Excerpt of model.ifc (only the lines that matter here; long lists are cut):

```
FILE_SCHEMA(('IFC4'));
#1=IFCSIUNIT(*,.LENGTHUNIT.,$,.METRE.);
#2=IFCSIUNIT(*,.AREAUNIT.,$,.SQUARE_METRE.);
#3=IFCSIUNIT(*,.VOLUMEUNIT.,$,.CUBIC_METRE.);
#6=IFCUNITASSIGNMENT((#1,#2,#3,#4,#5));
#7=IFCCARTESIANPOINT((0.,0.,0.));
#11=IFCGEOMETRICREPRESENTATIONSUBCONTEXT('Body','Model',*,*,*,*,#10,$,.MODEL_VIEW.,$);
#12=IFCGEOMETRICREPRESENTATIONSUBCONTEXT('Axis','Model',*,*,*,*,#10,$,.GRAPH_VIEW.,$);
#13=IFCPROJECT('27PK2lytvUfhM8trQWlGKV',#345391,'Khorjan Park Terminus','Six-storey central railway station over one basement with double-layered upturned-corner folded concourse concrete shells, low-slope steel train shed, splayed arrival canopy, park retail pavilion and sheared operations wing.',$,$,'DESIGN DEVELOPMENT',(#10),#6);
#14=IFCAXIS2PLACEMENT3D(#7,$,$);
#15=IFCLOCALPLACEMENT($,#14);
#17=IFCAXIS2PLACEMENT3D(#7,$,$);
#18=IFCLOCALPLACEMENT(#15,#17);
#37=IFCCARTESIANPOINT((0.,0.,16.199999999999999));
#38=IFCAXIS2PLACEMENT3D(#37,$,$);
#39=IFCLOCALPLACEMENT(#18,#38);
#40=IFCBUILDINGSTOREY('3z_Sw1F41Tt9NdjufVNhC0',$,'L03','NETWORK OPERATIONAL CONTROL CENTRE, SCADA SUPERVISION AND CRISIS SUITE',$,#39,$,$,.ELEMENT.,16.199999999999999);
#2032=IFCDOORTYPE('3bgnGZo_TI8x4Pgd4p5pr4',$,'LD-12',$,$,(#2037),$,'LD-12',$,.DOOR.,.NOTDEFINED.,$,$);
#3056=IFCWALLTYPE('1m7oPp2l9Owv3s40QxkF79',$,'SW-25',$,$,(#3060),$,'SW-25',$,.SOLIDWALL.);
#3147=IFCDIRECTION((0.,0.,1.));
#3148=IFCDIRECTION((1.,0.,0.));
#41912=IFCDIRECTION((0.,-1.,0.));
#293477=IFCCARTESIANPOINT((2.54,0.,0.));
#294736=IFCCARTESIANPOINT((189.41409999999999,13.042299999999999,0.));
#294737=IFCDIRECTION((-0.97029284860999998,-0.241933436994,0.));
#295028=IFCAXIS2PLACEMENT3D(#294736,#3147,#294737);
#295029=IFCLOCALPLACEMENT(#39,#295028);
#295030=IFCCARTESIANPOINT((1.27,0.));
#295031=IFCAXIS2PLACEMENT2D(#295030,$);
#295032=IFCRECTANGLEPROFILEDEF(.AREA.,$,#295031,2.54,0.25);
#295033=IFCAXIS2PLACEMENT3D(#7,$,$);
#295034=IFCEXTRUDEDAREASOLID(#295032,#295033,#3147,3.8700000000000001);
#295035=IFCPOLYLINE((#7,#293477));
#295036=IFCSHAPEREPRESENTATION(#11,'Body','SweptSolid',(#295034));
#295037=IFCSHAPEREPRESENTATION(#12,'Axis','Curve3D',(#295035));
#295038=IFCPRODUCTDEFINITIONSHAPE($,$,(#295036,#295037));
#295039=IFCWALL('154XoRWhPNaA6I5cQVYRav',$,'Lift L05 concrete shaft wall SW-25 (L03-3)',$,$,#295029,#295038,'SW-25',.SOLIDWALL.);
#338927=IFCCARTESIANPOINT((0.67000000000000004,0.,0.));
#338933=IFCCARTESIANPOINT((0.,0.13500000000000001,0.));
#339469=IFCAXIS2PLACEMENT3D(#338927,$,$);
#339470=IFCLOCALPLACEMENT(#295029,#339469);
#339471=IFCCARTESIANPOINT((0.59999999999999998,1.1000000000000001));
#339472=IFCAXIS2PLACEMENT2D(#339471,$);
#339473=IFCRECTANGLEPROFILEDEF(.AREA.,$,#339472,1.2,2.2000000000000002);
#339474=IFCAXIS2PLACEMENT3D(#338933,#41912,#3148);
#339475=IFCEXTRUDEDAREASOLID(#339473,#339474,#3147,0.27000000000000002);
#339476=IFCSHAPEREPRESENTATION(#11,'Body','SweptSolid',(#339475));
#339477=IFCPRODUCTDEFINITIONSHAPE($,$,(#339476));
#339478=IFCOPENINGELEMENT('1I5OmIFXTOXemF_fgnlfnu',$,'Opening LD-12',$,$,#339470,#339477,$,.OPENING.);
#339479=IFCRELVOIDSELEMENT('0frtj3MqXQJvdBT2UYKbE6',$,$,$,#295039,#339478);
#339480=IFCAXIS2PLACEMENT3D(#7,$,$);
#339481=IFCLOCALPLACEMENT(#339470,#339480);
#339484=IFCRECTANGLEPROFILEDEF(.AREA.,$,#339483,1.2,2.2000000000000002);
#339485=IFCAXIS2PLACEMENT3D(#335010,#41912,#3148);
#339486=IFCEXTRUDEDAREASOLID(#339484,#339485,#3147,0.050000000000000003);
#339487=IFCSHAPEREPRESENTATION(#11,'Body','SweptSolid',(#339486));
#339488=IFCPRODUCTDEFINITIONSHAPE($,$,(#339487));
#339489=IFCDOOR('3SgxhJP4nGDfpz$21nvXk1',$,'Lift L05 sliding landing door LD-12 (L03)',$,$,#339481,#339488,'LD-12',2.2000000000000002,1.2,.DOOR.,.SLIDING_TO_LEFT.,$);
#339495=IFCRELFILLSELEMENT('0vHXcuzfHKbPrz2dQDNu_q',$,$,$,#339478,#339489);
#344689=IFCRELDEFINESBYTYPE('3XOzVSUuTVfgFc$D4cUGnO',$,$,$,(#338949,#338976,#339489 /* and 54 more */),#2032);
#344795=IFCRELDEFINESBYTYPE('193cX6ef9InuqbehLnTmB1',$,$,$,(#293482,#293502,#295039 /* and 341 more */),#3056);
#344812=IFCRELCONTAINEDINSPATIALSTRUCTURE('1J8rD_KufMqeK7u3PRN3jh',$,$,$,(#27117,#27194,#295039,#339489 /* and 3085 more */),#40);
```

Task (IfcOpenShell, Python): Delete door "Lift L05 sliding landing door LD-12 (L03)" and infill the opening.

```python
import ifcopenshell
import ifcopenshell.api.feature
import ifcopenshell.api.root
import ifcopenshell.geom
import ifcopenshell.util.shape

model = ifcopenshell.open("model.ifc")
settings = ifcopenshell.geom.settings()


def volume(element):
    """Net volume in cubic metres, openings subtracted."""
    shape = ifcopenshell.geom.create_shape(settings, element)
    return ifcopenshell.util.shape.get_volume(shape.geometry)


door = model.by_id(339489)
opening = door.FillsVoids[0].RelatingOpeningElement
wall = opening.VoidsElements[0].RelatingBuildingElement
before = volume(wall)

ifcopenshell.api.root.remove_product(model, product=door)
ifcopenshell.api.feature.remove_feature(model, feature=opening)

after = volume(wall)

print(f"wall volume {before:.3f} -> {after:.3f} m3")

model.write("model-out.ifc")
```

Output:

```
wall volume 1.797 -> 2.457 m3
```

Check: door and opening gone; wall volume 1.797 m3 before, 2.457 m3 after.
